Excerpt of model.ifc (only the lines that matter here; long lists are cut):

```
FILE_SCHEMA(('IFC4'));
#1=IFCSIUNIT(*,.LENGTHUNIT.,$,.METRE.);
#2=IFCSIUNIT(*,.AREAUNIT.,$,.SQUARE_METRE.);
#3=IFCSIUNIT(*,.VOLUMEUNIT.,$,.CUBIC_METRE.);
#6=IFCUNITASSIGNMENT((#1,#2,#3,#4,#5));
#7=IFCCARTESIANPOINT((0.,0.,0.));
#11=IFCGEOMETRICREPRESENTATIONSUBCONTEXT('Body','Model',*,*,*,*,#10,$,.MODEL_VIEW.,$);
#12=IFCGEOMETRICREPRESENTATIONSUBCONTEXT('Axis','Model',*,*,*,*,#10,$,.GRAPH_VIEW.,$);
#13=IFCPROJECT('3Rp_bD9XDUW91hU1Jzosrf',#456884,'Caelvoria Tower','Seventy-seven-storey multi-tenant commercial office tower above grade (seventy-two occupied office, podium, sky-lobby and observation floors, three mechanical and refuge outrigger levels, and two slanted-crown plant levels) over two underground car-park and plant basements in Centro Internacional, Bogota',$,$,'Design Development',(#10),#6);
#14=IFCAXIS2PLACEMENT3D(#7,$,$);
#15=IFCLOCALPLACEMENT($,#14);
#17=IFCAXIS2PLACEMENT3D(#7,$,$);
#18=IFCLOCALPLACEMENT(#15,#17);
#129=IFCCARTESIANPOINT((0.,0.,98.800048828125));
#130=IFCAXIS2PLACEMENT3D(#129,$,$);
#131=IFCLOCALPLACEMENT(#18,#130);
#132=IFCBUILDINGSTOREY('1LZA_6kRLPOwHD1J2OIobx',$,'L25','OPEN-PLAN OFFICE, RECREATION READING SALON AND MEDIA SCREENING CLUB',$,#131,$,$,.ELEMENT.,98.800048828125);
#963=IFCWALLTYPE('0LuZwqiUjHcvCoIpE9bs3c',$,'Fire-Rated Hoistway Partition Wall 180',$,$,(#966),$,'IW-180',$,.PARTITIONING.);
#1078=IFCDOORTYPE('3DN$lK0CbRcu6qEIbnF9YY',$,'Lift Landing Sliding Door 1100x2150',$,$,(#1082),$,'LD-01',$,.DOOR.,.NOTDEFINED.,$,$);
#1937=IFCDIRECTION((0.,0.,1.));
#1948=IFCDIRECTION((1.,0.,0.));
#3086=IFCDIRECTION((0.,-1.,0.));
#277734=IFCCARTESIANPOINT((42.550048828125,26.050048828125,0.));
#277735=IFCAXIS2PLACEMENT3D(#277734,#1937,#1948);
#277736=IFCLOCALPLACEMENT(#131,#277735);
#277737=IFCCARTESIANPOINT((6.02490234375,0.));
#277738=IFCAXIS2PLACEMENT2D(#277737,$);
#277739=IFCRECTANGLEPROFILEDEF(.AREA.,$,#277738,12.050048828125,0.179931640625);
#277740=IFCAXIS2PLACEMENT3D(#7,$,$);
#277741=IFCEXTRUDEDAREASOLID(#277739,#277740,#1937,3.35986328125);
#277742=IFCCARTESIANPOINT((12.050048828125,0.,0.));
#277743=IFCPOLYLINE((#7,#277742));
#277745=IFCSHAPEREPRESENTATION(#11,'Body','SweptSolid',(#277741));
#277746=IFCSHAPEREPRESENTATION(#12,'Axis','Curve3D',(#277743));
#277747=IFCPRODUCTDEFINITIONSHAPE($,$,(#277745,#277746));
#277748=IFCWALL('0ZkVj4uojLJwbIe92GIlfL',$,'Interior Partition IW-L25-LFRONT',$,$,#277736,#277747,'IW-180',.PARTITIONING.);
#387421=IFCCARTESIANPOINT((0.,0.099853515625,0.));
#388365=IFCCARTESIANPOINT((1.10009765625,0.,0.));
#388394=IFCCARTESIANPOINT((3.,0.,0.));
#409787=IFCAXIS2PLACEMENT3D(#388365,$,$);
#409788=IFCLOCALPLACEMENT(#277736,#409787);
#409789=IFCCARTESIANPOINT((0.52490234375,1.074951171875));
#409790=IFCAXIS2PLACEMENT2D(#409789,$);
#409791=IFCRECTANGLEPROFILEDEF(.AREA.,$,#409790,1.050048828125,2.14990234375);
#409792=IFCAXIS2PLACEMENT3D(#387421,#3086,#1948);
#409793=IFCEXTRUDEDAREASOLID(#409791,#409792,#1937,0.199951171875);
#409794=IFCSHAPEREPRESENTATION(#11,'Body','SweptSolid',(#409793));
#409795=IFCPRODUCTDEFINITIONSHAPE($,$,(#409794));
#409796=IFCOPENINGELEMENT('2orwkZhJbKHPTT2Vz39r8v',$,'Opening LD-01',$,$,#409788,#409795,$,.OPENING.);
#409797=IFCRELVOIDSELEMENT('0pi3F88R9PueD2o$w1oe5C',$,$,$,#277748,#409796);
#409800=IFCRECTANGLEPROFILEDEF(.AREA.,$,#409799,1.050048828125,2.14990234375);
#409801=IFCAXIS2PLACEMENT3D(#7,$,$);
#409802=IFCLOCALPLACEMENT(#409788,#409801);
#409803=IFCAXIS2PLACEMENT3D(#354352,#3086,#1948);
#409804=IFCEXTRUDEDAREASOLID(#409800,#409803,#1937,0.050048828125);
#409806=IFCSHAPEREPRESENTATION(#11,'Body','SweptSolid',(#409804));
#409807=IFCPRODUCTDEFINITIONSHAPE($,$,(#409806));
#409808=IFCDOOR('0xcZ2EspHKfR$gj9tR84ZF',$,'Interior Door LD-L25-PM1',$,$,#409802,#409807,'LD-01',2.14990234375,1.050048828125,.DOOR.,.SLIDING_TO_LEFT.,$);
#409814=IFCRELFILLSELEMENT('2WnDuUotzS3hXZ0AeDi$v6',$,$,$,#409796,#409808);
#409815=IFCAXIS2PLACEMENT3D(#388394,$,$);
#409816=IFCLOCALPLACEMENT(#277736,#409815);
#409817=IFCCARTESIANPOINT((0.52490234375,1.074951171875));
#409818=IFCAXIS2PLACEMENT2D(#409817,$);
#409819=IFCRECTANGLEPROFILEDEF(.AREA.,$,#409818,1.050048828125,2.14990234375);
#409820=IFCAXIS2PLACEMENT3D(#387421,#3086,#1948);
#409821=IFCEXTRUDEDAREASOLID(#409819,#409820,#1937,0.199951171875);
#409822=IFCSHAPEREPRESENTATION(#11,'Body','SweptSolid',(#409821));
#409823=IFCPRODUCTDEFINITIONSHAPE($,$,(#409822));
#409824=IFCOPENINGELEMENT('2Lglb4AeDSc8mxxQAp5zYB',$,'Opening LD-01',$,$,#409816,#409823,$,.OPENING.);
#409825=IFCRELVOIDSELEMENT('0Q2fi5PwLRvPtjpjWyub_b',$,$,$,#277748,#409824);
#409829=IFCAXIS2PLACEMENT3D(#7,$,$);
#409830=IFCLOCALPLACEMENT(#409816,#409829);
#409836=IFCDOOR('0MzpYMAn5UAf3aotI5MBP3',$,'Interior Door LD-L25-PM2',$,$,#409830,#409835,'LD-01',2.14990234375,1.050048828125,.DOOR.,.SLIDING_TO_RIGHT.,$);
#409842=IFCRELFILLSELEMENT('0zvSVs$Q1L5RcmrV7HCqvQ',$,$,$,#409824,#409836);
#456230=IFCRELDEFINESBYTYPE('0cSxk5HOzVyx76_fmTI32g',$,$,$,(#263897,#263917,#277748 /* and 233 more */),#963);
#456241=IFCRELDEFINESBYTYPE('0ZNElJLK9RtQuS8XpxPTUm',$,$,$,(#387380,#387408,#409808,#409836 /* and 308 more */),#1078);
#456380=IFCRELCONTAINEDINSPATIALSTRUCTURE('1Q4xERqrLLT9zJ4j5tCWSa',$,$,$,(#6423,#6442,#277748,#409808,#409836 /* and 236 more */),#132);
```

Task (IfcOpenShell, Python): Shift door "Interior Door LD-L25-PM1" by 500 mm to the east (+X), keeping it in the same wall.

```python
import ifcopenshell
import ifcopenshell.api.geometry
import ifcopenshell.util.placement

model = ifcopenshell.open("model.ifc")

door = model.by_guid("0xcZ2EspHKfR$gj9tR84ZF")
opening = door.FillsVoids[0].RelatingOpeningElement
wall = opening.VoidsElements[0].RelatingBuildingElement

wall_matrix = ifcopenshell.util.placement.get_local_placement(wall.ObjectPlacement)
shift = wall_matrix[:3, 0] * 0.5
before = ifcopenshell.util.placement.get_local_placement(door.ObjectPlacement)[:3, 3].copy()

# The door is placed relative to its opening, so it follows when the opening moves.
matrix = ifcopenshell.util.placement.get_local_placement(opening.ObjectPlacement)
matrix[:3, 3] += shift
ifcopenshell.api.geometry.edit_object_placement(
    model, product=opening, matrix=matrix, is_si=False, should_transform_children=True
)

after = ifcopenshell.util.placement.get_local_placement(door.ObjectPlacement)[:3, 3]
print("door moved by", (after - before).round(3) + 0.0)

model.write("model_updated.ifc")
```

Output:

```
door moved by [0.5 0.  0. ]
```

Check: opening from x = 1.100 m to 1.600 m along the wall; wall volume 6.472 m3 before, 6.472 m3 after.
